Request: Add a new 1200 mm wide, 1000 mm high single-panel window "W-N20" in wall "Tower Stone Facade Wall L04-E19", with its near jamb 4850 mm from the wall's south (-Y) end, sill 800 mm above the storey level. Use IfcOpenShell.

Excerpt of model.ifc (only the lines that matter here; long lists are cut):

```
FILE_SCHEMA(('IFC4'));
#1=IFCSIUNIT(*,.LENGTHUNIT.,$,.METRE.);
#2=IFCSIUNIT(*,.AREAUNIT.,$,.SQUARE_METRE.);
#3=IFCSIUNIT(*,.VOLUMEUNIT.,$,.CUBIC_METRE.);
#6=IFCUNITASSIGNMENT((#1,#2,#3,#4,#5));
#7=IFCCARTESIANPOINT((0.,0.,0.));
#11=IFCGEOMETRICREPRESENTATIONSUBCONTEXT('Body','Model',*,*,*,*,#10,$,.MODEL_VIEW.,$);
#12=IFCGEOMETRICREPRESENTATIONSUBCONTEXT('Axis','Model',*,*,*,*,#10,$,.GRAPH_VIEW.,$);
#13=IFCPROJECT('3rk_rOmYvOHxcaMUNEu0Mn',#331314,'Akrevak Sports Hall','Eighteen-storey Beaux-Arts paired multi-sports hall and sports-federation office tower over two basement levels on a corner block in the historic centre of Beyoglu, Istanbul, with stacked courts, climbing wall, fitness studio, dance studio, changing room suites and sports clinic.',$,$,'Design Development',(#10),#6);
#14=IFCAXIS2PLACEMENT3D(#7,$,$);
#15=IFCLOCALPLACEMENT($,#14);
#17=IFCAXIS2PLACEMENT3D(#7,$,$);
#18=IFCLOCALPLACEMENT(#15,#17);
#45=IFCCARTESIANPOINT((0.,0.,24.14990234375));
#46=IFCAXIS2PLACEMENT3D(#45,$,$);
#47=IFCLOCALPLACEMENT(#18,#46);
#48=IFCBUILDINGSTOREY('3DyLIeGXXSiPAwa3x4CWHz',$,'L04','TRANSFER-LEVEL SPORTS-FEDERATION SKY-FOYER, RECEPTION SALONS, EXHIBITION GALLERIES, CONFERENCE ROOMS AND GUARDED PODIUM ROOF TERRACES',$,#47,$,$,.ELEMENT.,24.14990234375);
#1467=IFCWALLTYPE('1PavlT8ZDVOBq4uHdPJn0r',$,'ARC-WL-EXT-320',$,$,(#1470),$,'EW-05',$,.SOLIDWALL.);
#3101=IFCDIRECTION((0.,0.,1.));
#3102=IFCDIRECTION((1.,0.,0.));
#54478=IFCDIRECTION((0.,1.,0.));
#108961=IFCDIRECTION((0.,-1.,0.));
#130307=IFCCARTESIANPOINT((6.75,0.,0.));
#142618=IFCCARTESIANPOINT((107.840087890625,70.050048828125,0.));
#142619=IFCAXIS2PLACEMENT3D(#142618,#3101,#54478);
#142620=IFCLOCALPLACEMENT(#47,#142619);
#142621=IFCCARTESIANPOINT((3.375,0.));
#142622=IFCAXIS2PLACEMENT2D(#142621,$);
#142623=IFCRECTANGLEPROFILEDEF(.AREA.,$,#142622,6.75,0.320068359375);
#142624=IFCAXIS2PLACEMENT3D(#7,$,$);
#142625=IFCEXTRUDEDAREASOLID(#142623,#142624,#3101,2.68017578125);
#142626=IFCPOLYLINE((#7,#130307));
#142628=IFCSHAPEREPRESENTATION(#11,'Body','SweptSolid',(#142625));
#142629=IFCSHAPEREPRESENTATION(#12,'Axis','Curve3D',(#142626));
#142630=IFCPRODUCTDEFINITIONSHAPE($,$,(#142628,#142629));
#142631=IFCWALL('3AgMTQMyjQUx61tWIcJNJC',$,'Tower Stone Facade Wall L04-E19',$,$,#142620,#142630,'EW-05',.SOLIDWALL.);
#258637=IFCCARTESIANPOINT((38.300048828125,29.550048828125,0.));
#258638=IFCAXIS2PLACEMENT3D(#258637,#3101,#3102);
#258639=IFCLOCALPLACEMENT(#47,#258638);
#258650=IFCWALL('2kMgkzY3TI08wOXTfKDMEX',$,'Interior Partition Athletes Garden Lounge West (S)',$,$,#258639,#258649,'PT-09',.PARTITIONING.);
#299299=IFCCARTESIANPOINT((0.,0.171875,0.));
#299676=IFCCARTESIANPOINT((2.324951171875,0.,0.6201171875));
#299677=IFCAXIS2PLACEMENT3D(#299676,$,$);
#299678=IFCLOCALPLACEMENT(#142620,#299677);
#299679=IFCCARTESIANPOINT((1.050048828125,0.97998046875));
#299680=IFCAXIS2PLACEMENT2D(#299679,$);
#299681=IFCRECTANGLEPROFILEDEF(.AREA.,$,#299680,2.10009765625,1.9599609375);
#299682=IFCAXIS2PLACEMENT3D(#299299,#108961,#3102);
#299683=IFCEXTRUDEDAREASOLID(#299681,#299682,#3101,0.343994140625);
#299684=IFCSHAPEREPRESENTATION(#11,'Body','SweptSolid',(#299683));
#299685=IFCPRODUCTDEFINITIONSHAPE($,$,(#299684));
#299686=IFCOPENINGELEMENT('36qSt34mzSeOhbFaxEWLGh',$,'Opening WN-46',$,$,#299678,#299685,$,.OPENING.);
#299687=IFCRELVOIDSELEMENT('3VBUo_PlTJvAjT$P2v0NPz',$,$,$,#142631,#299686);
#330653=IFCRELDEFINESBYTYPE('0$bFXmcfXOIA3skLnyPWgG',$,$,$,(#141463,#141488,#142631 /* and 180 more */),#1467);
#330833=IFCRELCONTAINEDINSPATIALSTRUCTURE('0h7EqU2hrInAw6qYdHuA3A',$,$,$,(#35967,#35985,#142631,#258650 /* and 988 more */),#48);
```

```python
import numpy as np
import ifcopenshell
import ifcopenshell.api.feature
import ifcopenshell.api.geometry
import ifcopenshell.api.root
import ifcopenshell.api.spatial
import ifcopenshell.geom
import ifcopenshell.util.element
import ifcopenshell.util.placement
import ifcopenshell.util.representation
import ifcopenshell.util.shape
import ifcopenshell.util.unit

model = ifcopenshell.open("model.ifc")
unit_scale = ifcopenshell.util.unit.calculate_unit_scale(model)
settings = ifcopenshell.geom.settings()


def volume(element):
    """Net volume in cubic metres, openings subtracted."""
    shape = ifcopenshell.geom.create_shape(settings, element)
    return ifcopenshell.util.shape.get_volume(shape.geometry)


wall = model.by_guid("3AgMTQMyjQUx61tWIcJNJC")
storey = ifcopenshell.util.element.get_container(wall, ifc_class="IfcBuildingStorey")
context = ifcopenshell.util.representation.get_context(model, "Model", "Body", "MODEL_VIEW")
before = volume(wall)

width, height, from_end, sill = 1.2, 1, 4.85, 0.8  # metres

# The wall runs along its own X axis, and the end named is its -X end.
wall_shape = ifcopenshell.geom.create_shape(settings, wall)
x, y, z = ifcopenshell.util.shape.get_vertices(wall_shape.geometry).T
start = x.min() + from_end
face, thickness = float(y.min()), float(y.max() - y.min())
wall_matrix = ifcopenshell.util.placement.get_local_placement(wall.ObjectPlacement)
level = ifcopenshell.util.placement.get_local_placement(storey.ObjectPlacement)[2, 3]


def in_wall(x, y):
    """Placement at x, y metres in the wall's axes, at sill height."""
    matrix = wall_matrix.copy()
    matrix[:, 3] = wall_matrix @ np.array([x / unit_scale, y / unit_scale, 0.0, 1.0])
    matrix[2, 3] = level + sill / unit_scale
    return matrix


# Opening: a box that overshoots both wall faces by 50 mm.
opening = ifcopenshell.api.root.create_entity(model, ifc_class="IfcOpeningElement", predefined_type="OPENING")
box = ifcopenshell.api.geometry.add_wall_representation(
    model, context=context, length=width, height=height, thickness=thickness + 0.1
)
ifcopenshell.api.geometry.assign_representation(model, product=opening, representation=box)
ifcopenshell.api.geometry.edit_object_placement(model, product=opening, matrix=in_wall(start, face - 0.05), is_si=False)
ifcopenshell.api.feature.add_feature(model, feature=opening, element=wall)

window = ifcopenshell.api.root.create_entity(model, ifc_class="IfcWindow", name="W-N20", predefined_type="WINDOW")
window.OverallWidth, window.OverallHeight = width / unit_scale, height / unit_scale
window.PartitioningType = "SINGLE_PANEL"
body = ifcopenshell.api.geometry.add_window_representation(
    model,
    context=context,
    overall_width=window.OverallWidth,
    overall_height=window.OverallHeight,
    partition_type="SINGLE_PANEL",
)
ifcopenshell.api.geometry.assign_representation(model, product=window, representation=body)
ifcopenshell.api.spatial.assign_container(model, products=[window], relating_structure=storey)
ifcopenshell.api.feature.add_filling(model, opening=opening, element=window)

# Centre the window in the wall's thickness.
ifcopenshell.api.geometry.edit_object_placement(model, product=window, matrix=in_wall(start, face), is_si=False)
window_shape = ifcopenshell.geom.create_shape(settings, window)
depth = ifcopenshell.util.shape.get_vertices(window_shape.geometry)[:, 1]
offset = face + thickness / 2 - (depth.min() + depth.max()) / 2
ifcopenshell.api.geometry.edit_object_placement(model, product=window, matrix=in_wall(start, offset), is_si=False)

after = volume(wall)

print(f"wall volume {before:.3f} -> {after:.3f} m3")

model.write("model_rev.ifc")
```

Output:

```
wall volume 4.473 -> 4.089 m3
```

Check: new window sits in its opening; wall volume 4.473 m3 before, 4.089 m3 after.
